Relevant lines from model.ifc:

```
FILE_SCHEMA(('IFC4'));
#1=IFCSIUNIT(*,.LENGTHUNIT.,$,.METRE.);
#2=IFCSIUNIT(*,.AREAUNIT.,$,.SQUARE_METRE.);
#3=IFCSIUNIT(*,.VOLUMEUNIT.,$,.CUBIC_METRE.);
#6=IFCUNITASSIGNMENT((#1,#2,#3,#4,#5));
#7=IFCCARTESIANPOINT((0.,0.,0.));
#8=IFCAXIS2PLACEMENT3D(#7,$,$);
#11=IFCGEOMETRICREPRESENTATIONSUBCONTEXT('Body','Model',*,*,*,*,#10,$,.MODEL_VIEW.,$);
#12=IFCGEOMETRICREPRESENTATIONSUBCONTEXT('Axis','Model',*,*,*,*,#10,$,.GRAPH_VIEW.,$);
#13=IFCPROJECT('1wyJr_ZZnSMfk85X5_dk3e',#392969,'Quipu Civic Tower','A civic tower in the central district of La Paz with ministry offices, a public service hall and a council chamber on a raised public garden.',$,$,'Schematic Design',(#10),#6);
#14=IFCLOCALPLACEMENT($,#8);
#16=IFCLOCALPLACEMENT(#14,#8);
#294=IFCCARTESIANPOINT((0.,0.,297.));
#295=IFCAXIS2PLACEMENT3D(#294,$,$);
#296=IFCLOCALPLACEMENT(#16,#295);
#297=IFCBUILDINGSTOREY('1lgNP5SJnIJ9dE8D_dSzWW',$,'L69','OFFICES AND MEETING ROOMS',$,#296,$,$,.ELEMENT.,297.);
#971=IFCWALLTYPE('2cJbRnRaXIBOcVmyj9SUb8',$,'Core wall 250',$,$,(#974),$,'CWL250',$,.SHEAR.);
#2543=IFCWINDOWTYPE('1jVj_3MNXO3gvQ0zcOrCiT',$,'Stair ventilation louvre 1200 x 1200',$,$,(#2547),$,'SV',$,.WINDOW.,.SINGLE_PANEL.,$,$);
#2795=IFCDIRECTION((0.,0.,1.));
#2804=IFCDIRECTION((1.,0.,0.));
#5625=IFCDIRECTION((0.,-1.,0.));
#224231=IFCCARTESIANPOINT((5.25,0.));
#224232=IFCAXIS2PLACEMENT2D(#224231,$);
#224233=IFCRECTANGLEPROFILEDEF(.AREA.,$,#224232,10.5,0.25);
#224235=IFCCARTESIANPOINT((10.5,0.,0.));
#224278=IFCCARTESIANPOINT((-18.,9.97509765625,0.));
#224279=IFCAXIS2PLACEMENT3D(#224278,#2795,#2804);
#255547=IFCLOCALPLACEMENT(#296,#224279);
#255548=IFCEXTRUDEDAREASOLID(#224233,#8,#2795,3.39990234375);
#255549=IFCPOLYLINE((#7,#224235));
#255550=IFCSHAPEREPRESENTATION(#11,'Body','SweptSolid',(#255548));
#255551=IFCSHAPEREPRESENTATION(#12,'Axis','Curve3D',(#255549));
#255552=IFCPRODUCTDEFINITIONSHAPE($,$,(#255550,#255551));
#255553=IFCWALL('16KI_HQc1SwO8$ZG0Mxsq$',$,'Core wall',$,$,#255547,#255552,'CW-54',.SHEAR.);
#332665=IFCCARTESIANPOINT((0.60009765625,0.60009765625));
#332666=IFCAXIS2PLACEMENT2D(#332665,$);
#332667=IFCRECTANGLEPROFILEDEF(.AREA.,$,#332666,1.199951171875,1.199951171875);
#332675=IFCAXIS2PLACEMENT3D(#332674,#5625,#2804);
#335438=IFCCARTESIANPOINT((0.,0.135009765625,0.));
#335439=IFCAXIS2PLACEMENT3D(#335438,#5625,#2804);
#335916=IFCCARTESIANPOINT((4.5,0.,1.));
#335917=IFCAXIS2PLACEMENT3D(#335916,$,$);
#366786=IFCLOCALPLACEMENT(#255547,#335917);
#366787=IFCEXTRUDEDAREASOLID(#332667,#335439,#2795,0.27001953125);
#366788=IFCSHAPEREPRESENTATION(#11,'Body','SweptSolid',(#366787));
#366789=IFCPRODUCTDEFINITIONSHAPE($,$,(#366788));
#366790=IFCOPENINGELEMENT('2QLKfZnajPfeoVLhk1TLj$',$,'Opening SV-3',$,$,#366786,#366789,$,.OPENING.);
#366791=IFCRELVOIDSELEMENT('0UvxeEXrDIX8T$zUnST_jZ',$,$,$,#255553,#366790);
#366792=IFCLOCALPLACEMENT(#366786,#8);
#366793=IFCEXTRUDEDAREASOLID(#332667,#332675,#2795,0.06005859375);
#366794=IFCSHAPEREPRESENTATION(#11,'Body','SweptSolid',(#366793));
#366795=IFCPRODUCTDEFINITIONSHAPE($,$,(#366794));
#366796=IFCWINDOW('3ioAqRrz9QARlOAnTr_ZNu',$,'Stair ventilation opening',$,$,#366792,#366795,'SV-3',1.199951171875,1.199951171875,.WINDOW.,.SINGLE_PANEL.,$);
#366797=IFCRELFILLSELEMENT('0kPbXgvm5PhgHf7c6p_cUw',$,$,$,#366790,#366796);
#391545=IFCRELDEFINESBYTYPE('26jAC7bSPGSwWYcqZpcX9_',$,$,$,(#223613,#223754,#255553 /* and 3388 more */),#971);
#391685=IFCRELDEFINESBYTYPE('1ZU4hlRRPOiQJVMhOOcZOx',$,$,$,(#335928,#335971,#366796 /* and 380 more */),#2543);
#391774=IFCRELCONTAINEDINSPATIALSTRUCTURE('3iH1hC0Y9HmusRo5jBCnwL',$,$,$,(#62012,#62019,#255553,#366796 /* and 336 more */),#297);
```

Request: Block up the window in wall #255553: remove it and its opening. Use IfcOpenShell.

```python
import ifcopenshell
import ifcopenshell.api.feature
import ifcopenshell.api.root
import ifcopenshell.geom
import ifcopenshell.util.shape

model = ifcopenshell.open("model.ifc")
settings = ifcopenshell.geom.settings()


def volume(element):
    """Net volume in cubic metres, openings subtracted."""
    shape = ifcopenshell.geom.create_shape(settings, element)
    return ifcopenshell.util.shape.get_volume(shape.geometry)


window = model.by_id(366796)
opening = window.FillsVoids[0].RelatingOpeningElement
wall = opening.VoidsElements[0].RelatingBuildingElement
before = volume(wall)

ifcopenshell.api.root.remove_product(model, product=window)
ifcopenshell.api.feature.remove_feature(model, feature=opening)

after = volume(wall)

print(f"wall volume {before:.3f} -> {after:.3f} m3")

model.write("model_updated.ifc")
```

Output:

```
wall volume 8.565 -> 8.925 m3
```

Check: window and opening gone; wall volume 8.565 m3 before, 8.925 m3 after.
